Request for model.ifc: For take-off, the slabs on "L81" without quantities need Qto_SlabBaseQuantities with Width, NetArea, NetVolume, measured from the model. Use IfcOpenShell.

First a look at what the model holds.

```python
import ifcopenshell
import ifcopenshell.util.element
import ifcopenshell.util.unit

model = ifcopenshell.open("model.ifc")
print(model.schema)
for unit_type in ("LENGTHUNIT", "AREAUNIT", "VOLUMEUNIT"):
    print(unit_type, ifcopenshell.util.unit.calculate_unit_scale(model, unit_type))
storey = next(s for s in model.by_type("IfcBuildingStorey") if s.Name == "L81")
slabs = [e for e in ifcopenshell.util.element.get_decomposition(storey) if e.is_a("IfcSlab")]
for e in sorted(slabs, key=lambda e: e.id()):
    print(e.id(), e.is_a(), e.Name, list(ifcopenshell.util.element.get_psets(e, qtos_only=True)), sep=" | ")
```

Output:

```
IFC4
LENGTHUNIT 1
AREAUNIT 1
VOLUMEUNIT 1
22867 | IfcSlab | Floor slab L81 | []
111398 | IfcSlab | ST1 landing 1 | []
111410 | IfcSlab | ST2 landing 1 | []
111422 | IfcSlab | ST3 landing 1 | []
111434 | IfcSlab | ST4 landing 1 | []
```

```python
import ifcopenshell
import ifcopenshell.api.pset
import ifcopenshell.geom
import ifcopenshell.util.element
import ifcopenshell.util.shape
import ifcopenshell.util.unit

model = ifcopenshell.open("model.ifc")
unit_scale = ifcopenshell.util.unit.calculate_unit_scale(model)
area_scale = ifcopenshell.util.unit.calculate_unit_scale(model, "AREAUNIT")
volume_scale = ifcopenshell.util.unit.calculate_unit_scale(model, "VOLUMEUNIT")
settings = ifcopenshell.geom.settings()

storey = next(s for s in model.by_type("IfcBuildingStorey") if s.Name == "L81")
slabs = [e for e in ifcopenshell.util.element.get_decomposition(storey) if e.is_a("IfcSlab")]

for e in sorted(slabs, key=lambda e: e.id()):
    if ifcopenshell.util.element.get_psets(e, qtos_only=True, should_inherit=False):
        continue
    # Geometry comes back in metres, in the element's own axes.
    shape = ifcopenshell.geom.create_shape(settings, e)
    values = {
        "Width": ifcopenshell.util.shape.get_z(shape.geometry) / unit_scale,
        "NetArea": ifcopenshell.util.shape.get_footprint_area(shape.geometry) / area_scale,
        "NetVolume": ifcopenshell.util.shape.get_volume(shape.geometry) / volume_scale,
    }
    qto = ifcopenshell.api.pset.add_qto(model, product=e, name="Qto_SlabBaseQuantities")
    ifcopenshell.api.pset.edit_qto(model, qto=qto, properties=values)
    print(e.id(), {k: round(v, 3) for k, v in values.items()})

model.write("model_edited.ifc")
```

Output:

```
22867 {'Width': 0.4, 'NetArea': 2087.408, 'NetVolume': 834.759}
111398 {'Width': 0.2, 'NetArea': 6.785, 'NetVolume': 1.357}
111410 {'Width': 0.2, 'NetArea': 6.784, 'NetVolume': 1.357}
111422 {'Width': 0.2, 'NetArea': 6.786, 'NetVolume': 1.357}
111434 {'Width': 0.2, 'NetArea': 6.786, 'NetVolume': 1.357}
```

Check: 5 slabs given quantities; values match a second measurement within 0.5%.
